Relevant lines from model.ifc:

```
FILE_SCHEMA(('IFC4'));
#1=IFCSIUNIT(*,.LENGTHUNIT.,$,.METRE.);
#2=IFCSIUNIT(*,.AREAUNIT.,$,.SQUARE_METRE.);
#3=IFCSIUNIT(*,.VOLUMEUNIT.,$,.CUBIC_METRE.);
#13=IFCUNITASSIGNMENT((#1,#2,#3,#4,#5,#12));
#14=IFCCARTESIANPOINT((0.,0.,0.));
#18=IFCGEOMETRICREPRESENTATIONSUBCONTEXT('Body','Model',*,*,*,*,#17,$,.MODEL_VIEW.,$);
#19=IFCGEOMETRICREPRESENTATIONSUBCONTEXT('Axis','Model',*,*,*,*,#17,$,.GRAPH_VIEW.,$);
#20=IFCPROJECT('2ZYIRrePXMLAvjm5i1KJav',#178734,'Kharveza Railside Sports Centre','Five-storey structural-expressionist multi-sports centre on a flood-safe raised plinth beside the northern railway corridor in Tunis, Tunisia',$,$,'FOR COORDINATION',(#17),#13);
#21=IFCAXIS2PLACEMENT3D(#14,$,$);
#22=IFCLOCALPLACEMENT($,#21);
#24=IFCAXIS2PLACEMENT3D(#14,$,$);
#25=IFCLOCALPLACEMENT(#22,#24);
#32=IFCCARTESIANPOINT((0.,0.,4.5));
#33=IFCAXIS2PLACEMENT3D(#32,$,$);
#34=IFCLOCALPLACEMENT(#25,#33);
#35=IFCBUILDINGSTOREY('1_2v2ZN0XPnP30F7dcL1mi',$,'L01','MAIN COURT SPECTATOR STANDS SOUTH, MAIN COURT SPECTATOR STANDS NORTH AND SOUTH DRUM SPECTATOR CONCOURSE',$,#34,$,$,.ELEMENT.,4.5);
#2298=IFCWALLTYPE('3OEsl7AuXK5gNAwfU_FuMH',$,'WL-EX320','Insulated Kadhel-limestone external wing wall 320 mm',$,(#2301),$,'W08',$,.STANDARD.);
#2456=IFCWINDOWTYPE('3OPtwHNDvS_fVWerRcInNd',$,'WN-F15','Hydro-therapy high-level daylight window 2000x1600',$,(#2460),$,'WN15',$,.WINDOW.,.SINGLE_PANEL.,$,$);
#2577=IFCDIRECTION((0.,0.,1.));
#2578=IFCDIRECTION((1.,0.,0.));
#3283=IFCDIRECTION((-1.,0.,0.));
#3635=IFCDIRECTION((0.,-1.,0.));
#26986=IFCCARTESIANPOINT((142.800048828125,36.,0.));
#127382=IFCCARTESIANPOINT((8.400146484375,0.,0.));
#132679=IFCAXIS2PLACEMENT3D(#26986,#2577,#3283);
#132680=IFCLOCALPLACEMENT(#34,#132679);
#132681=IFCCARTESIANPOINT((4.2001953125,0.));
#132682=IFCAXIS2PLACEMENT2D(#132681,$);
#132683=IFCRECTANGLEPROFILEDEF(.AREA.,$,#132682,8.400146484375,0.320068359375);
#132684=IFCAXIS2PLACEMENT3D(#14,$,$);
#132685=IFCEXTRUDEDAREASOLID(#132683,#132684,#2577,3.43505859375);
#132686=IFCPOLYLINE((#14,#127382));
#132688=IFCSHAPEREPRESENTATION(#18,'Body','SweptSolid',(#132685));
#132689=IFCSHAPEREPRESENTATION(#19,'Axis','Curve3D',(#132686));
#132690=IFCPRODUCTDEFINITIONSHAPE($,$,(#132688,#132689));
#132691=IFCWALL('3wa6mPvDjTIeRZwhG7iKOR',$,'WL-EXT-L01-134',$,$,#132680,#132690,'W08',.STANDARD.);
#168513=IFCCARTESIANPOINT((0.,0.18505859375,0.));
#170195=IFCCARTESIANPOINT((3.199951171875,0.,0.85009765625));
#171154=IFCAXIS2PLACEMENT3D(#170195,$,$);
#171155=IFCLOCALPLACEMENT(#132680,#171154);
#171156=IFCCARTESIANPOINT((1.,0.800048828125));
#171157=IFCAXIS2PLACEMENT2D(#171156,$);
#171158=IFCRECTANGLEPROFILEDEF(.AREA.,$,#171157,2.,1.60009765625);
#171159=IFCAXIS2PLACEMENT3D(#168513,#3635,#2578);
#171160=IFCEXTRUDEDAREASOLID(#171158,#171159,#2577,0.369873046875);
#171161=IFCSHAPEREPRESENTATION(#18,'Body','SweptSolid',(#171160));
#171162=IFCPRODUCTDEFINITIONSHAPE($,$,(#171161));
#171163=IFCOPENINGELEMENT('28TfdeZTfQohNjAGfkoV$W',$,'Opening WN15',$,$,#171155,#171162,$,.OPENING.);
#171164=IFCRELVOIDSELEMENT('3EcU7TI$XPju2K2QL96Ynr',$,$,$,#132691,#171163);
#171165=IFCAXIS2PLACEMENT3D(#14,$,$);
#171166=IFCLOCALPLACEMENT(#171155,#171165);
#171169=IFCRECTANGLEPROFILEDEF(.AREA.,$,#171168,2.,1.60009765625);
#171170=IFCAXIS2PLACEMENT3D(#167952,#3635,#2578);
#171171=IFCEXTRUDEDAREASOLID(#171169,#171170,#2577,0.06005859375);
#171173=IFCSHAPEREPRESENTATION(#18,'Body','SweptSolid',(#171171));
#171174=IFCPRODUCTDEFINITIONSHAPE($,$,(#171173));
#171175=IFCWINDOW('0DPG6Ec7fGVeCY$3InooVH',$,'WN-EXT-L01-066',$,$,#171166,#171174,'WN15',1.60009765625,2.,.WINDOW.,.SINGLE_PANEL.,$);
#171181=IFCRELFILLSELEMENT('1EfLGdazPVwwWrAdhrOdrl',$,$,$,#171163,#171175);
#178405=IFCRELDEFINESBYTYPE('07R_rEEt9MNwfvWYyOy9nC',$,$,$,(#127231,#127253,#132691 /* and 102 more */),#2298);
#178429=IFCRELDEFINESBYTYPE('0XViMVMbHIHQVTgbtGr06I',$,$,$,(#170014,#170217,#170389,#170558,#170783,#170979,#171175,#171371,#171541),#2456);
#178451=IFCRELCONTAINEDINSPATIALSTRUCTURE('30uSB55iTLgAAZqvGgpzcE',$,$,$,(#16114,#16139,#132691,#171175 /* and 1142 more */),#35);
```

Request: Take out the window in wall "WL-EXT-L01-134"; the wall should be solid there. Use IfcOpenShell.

```python
import ifcopenshell
import ifcopenshell.api.feature
import ifcopenshell.api.root
import ifcopenshell.geom
import ifcopenshell.util.shape

model = ifcopenshell.open("model.ifc")
settings = ifcopenshell.geom.settings()


def volume(element):
    """Net volume in cubic metres, openings subtracted."""
    shape = ifcopenshell.geom.create_shape(settings, element)
    return ifcopenshell.util.shape.get_volume(shape.geometry)


window = model.by_guid("0DPG6Ec7fGVeCY$3InooVH")
opening = window.FillsVoids[0].RelatingOpeningElement
wall = opening.VoidsElements[0].RelatingBuildingElement
before = volume(wall)

ifcopenshell.api.root.remove_product(model, product=window)
ifcopenshell.api.feature.remove_feature(model, feature=opening)

after = volume(wall)

print(f"wall volume {before:.3f} -> {after:.3f} m3")

model.write("model_updated.ifc")
```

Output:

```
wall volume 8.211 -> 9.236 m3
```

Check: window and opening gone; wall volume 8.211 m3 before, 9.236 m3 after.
